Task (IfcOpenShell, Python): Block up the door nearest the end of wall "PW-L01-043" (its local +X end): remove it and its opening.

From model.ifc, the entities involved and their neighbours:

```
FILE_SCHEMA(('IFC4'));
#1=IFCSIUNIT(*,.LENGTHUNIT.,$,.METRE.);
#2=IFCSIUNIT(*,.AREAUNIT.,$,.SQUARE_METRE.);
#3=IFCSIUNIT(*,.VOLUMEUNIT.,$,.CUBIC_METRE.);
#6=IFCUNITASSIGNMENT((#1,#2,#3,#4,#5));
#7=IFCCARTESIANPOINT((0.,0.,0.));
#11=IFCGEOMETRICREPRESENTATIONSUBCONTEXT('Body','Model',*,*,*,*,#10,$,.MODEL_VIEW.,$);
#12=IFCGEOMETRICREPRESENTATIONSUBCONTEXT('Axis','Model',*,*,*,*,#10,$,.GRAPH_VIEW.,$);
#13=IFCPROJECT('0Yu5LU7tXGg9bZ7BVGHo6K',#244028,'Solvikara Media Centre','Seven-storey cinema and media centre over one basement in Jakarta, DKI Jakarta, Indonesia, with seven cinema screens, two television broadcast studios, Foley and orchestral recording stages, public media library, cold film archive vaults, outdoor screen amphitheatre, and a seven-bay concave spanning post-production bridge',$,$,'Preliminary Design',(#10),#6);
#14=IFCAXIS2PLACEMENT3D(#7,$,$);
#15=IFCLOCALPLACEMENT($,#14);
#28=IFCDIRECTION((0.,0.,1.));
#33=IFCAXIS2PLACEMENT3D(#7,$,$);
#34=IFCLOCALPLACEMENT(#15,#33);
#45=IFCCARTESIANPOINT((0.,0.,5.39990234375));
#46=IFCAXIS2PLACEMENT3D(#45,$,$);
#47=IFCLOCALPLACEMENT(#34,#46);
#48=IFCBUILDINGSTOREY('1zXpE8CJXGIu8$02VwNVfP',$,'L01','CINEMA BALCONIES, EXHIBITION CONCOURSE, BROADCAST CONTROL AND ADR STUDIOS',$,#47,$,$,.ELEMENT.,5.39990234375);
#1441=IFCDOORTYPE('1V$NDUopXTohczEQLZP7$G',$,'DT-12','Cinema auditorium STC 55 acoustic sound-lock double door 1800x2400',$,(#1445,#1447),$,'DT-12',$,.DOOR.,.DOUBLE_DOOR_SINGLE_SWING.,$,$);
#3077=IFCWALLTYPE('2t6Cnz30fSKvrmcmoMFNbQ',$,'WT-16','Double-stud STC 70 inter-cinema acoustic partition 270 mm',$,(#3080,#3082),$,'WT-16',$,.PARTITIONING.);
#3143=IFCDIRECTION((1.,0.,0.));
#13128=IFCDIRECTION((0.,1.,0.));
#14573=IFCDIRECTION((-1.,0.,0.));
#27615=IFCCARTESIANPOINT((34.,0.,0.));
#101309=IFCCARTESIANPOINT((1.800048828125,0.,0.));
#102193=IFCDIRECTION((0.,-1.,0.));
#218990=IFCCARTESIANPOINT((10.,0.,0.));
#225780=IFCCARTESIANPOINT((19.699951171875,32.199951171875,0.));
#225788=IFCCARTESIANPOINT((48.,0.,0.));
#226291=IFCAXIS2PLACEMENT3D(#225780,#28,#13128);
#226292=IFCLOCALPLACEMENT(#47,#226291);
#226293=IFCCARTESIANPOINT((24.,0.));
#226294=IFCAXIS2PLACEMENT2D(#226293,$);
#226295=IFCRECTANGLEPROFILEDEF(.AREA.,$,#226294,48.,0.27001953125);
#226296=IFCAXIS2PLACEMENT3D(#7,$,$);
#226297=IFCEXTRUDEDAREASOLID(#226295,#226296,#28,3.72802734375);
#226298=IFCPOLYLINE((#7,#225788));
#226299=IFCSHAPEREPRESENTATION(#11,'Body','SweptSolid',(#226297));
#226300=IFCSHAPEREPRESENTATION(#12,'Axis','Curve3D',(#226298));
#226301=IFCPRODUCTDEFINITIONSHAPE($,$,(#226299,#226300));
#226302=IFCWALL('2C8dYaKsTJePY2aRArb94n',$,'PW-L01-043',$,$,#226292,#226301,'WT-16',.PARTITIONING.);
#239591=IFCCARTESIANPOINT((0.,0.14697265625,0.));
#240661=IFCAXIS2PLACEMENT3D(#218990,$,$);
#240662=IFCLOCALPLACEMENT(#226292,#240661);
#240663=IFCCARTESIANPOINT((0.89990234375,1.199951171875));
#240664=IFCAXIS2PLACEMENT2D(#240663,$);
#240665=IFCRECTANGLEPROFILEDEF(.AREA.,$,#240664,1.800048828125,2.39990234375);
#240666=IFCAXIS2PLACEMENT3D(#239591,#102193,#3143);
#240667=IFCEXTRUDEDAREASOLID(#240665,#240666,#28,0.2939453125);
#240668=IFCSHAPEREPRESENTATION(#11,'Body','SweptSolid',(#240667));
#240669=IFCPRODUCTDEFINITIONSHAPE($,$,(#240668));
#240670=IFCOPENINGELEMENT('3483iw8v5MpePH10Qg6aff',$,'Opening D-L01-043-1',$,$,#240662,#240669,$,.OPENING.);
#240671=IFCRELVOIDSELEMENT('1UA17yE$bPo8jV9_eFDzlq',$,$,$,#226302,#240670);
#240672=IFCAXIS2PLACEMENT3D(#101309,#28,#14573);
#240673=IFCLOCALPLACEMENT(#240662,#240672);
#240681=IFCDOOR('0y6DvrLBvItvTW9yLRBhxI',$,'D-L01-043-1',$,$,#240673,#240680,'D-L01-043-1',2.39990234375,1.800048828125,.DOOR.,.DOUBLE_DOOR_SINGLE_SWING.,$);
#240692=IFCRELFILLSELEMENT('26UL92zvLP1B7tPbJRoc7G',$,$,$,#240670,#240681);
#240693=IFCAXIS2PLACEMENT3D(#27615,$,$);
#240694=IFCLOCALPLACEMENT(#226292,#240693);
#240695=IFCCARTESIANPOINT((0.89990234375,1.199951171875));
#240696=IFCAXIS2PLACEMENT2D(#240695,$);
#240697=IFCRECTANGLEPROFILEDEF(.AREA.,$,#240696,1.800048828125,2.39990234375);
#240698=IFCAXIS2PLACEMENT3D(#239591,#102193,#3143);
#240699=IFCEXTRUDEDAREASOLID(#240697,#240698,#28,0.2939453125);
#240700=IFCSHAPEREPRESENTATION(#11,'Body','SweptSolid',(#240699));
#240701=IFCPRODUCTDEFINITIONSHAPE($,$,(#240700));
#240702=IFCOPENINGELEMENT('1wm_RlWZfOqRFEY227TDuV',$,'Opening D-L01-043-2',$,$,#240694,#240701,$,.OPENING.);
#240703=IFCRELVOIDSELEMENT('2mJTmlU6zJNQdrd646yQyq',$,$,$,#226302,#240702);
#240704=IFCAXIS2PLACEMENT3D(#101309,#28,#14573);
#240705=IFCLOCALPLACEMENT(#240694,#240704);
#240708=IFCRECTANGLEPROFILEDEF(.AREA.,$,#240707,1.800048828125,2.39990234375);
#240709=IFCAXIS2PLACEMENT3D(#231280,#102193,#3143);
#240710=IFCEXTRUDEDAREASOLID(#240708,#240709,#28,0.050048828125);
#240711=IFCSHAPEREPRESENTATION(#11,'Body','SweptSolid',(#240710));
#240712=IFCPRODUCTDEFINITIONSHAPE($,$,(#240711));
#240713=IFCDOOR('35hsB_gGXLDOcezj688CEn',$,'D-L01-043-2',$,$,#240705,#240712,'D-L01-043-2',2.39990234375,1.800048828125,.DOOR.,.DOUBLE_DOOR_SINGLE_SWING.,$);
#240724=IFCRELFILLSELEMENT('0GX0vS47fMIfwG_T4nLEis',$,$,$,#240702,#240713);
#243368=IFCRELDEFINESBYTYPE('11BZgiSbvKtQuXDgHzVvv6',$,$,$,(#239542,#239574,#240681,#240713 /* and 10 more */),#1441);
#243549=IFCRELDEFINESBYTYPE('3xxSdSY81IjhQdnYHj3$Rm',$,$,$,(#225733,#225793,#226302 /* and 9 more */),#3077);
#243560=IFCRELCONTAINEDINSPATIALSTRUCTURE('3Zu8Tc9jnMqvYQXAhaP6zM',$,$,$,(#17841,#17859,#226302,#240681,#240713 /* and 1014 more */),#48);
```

```python
import ifcopenshell
import ifcopenshell.api.feature
import ifcopenshell.api.root
import ifcopenshell.geom
import ifcopenshell.util.shape

model = ifcopenshell.open("model.ifc")
settings = ifcopenshell.geom.settings()


def volume(element):
    """Net volume in cubic metres, openings subtracted."""
    shape = ifcopenshell.geom.create_shape(settings, element)
    return ifcopenshell.util.shape.get_volume(shape.geometry)


door = model.by_guid("35hsB_gGXLDOcezj688CEn")
opening = door.FillsVoids[0].RelatingOpeningElement
wall = opening.VoidsElements[0].RelatingBuildingElement
before = volume(wall)

ifcopenshell.api.root.remove_product(model, product=door)
ifcopenshell.api.feature.remove_feature(model, feature=opening)

after = volume(wall)

print(f"wall volume {before:.3f} -> {after:.3f} m3")

model.write("model_rev.ifc")
```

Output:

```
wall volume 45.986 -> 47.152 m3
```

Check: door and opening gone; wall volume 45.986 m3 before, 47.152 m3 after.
